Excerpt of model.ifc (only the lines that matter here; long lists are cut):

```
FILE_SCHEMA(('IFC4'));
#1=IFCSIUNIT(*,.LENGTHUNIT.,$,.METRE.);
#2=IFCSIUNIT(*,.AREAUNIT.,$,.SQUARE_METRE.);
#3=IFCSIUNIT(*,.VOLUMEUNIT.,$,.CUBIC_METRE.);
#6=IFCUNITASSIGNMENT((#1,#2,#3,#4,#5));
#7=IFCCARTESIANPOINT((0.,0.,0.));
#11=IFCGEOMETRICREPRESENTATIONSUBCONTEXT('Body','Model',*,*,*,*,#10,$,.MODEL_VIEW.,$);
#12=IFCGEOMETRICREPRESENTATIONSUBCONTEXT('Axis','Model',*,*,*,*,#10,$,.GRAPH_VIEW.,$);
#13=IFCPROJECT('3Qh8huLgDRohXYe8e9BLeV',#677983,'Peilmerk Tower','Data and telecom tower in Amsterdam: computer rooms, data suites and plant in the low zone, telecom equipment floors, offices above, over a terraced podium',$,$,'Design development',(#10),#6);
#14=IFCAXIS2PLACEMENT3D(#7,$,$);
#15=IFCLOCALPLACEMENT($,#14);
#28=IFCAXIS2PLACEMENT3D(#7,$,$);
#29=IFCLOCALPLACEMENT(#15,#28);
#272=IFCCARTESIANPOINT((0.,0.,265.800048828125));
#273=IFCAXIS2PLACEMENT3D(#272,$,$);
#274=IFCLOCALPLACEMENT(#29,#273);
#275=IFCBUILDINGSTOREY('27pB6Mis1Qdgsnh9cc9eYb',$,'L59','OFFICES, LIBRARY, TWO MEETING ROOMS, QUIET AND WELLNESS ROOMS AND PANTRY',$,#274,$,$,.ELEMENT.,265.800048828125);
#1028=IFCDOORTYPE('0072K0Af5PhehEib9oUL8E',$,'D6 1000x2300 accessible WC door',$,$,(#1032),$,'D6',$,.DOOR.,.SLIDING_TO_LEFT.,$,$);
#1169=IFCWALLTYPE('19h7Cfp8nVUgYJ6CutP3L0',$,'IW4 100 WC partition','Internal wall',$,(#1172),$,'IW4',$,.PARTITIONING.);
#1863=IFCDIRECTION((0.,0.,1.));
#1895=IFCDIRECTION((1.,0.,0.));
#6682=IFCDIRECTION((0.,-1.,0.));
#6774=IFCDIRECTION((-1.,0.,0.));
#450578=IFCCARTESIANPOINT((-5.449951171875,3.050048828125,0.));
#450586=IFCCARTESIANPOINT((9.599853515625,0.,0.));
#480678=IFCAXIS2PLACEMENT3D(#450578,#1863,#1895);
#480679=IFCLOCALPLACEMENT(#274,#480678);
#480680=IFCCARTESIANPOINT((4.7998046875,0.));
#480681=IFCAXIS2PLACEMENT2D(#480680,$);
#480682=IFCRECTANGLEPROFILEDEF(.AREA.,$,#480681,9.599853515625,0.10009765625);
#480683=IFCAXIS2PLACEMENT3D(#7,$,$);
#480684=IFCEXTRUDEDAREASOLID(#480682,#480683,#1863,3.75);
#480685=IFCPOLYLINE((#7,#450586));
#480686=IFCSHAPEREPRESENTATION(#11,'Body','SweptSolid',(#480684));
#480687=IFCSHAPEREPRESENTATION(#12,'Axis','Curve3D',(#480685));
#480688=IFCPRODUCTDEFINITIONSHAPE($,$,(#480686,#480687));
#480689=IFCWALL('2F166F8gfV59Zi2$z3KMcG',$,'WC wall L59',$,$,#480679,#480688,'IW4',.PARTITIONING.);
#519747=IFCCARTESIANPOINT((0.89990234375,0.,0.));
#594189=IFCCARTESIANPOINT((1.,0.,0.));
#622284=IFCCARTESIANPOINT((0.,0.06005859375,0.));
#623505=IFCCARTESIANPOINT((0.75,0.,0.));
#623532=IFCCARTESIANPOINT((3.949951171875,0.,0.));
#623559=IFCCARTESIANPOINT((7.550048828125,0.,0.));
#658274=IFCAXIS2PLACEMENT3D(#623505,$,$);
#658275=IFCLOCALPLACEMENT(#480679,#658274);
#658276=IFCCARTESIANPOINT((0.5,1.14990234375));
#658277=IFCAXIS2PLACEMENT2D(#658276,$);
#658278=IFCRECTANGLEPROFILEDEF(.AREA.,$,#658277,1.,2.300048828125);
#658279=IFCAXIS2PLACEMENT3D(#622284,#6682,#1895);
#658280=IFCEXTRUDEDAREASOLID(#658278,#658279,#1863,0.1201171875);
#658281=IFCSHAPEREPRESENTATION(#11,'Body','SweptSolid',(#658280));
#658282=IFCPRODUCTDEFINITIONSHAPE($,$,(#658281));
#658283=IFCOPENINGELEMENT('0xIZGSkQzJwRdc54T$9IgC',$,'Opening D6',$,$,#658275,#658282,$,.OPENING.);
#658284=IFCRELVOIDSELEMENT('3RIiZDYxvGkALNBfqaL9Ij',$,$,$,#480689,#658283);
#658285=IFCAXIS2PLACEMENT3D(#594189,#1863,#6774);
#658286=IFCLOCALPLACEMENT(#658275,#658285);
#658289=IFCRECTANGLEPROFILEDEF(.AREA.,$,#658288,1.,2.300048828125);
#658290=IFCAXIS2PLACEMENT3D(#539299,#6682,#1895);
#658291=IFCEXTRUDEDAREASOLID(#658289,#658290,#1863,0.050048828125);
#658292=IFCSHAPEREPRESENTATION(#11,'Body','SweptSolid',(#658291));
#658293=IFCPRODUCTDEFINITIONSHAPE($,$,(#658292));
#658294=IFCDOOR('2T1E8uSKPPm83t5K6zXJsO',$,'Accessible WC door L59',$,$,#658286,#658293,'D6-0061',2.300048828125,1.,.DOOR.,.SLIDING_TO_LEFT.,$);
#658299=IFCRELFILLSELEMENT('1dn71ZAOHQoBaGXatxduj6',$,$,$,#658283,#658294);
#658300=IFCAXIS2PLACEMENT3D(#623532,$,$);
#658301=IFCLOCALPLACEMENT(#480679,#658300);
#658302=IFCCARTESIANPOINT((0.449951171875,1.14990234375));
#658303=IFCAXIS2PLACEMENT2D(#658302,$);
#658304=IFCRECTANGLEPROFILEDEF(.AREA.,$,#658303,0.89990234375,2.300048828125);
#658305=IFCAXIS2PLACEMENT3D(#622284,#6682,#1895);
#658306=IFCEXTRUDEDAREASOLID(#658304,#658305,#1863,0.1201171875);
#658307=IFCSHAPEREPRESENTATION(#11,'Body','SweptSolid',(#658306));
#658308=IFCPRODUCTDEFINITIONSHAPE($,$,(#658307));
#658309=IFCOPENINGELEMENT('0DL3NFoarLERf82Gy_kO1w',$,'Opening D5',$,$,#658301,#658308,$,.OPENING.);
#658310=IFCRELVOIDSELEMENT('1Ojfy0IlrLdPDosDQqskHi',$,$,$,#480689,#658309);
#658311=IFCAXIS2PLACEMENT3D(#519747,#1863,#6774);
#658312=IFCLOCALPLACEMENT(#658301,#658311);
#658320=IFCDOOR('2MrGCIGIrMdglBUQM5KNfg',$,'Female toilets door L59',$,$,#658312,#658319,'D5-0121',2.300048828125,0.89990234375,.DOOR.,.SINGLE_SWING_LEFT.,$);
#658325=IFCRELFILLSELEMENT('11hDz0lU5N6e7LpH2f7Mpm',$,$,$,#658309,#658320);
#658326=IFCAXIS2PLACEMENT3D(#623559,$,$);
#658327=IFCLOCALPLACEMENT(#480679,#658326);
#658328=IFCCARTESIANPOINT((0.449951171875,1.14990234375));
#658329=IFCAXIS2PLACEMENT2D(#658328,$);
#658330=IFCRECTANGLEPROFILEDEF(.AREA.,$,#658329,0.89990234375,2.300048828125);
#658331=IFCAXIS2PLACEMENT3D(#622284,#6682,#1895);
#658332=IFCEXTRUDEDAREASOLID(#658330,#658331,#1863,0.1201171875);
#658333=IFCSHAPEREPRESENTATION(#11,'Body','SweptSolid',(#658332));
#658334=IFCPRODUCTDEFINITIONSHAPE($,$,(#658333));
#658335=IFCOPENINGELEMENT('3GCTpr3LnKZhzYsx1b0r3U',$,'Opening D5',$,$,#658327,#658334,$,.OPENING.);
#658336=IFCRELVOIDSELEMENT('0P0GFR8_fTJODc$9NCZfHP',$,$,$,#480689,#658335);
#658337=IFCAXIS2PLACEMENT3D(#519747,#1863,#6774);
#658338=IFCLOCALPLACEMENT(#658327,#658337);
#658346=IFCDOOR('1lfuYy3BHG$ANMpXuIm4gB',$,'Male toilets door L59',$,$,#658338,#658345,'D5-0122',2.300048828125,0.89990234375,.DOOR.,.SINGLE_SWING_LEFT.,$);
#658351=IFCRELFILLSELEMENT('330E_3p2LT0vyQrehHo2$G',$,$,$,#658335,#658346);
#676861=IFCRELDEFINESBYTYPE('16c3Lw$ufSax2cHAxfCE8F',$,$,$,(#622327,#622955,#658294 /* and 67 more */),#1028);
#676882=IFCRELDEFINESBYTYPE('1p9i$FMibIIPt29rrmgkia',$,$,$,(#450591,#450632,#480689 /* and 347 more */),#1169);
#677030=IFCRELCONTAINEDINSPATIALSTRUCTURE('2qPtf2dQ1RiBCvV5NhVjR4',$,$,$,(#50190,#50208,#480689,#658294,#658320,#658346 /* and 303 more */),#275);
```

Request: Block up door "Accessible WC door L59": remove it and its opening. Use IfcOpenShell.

```python
import ifcopenshell
import ifcopenshell.api.feature
import ifcopenshell.api.root
import ifcopenshell.geom
import ifcopenshell.util.shape

model = ifcopenshell.open("model.ifc")
settings = ifcopenshell.geom.settings()


def volume(element):
    """Net volume in cubic metres, openings subtracted."""
    shape = ifcopenshell.geom.create_shape(settings, element)
    return ifcopenshell.util.shape.get_volume(shape.geometry)


door = model.by_guid("2T1E8uSKPPm83t5K6zXJsO")
opening = door.FillsVoids[0].RelatingOpeningElement
wall = opening.VoidsElements[0].RelatingBuildingElement
before = volume(wall)

ifcopenshell.api.root.remove_product(model, product=door)
ifcopenshell.api.feature.remove_feature(model, feature=opening)

after = volume(wall)

print(f"wall volume {before:.3f} -> {after:.3f} m3")

model.write("model_updated.ifc")
```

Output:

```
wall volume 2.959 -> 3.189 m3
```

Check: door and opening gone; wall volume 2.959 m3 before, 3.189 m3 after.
